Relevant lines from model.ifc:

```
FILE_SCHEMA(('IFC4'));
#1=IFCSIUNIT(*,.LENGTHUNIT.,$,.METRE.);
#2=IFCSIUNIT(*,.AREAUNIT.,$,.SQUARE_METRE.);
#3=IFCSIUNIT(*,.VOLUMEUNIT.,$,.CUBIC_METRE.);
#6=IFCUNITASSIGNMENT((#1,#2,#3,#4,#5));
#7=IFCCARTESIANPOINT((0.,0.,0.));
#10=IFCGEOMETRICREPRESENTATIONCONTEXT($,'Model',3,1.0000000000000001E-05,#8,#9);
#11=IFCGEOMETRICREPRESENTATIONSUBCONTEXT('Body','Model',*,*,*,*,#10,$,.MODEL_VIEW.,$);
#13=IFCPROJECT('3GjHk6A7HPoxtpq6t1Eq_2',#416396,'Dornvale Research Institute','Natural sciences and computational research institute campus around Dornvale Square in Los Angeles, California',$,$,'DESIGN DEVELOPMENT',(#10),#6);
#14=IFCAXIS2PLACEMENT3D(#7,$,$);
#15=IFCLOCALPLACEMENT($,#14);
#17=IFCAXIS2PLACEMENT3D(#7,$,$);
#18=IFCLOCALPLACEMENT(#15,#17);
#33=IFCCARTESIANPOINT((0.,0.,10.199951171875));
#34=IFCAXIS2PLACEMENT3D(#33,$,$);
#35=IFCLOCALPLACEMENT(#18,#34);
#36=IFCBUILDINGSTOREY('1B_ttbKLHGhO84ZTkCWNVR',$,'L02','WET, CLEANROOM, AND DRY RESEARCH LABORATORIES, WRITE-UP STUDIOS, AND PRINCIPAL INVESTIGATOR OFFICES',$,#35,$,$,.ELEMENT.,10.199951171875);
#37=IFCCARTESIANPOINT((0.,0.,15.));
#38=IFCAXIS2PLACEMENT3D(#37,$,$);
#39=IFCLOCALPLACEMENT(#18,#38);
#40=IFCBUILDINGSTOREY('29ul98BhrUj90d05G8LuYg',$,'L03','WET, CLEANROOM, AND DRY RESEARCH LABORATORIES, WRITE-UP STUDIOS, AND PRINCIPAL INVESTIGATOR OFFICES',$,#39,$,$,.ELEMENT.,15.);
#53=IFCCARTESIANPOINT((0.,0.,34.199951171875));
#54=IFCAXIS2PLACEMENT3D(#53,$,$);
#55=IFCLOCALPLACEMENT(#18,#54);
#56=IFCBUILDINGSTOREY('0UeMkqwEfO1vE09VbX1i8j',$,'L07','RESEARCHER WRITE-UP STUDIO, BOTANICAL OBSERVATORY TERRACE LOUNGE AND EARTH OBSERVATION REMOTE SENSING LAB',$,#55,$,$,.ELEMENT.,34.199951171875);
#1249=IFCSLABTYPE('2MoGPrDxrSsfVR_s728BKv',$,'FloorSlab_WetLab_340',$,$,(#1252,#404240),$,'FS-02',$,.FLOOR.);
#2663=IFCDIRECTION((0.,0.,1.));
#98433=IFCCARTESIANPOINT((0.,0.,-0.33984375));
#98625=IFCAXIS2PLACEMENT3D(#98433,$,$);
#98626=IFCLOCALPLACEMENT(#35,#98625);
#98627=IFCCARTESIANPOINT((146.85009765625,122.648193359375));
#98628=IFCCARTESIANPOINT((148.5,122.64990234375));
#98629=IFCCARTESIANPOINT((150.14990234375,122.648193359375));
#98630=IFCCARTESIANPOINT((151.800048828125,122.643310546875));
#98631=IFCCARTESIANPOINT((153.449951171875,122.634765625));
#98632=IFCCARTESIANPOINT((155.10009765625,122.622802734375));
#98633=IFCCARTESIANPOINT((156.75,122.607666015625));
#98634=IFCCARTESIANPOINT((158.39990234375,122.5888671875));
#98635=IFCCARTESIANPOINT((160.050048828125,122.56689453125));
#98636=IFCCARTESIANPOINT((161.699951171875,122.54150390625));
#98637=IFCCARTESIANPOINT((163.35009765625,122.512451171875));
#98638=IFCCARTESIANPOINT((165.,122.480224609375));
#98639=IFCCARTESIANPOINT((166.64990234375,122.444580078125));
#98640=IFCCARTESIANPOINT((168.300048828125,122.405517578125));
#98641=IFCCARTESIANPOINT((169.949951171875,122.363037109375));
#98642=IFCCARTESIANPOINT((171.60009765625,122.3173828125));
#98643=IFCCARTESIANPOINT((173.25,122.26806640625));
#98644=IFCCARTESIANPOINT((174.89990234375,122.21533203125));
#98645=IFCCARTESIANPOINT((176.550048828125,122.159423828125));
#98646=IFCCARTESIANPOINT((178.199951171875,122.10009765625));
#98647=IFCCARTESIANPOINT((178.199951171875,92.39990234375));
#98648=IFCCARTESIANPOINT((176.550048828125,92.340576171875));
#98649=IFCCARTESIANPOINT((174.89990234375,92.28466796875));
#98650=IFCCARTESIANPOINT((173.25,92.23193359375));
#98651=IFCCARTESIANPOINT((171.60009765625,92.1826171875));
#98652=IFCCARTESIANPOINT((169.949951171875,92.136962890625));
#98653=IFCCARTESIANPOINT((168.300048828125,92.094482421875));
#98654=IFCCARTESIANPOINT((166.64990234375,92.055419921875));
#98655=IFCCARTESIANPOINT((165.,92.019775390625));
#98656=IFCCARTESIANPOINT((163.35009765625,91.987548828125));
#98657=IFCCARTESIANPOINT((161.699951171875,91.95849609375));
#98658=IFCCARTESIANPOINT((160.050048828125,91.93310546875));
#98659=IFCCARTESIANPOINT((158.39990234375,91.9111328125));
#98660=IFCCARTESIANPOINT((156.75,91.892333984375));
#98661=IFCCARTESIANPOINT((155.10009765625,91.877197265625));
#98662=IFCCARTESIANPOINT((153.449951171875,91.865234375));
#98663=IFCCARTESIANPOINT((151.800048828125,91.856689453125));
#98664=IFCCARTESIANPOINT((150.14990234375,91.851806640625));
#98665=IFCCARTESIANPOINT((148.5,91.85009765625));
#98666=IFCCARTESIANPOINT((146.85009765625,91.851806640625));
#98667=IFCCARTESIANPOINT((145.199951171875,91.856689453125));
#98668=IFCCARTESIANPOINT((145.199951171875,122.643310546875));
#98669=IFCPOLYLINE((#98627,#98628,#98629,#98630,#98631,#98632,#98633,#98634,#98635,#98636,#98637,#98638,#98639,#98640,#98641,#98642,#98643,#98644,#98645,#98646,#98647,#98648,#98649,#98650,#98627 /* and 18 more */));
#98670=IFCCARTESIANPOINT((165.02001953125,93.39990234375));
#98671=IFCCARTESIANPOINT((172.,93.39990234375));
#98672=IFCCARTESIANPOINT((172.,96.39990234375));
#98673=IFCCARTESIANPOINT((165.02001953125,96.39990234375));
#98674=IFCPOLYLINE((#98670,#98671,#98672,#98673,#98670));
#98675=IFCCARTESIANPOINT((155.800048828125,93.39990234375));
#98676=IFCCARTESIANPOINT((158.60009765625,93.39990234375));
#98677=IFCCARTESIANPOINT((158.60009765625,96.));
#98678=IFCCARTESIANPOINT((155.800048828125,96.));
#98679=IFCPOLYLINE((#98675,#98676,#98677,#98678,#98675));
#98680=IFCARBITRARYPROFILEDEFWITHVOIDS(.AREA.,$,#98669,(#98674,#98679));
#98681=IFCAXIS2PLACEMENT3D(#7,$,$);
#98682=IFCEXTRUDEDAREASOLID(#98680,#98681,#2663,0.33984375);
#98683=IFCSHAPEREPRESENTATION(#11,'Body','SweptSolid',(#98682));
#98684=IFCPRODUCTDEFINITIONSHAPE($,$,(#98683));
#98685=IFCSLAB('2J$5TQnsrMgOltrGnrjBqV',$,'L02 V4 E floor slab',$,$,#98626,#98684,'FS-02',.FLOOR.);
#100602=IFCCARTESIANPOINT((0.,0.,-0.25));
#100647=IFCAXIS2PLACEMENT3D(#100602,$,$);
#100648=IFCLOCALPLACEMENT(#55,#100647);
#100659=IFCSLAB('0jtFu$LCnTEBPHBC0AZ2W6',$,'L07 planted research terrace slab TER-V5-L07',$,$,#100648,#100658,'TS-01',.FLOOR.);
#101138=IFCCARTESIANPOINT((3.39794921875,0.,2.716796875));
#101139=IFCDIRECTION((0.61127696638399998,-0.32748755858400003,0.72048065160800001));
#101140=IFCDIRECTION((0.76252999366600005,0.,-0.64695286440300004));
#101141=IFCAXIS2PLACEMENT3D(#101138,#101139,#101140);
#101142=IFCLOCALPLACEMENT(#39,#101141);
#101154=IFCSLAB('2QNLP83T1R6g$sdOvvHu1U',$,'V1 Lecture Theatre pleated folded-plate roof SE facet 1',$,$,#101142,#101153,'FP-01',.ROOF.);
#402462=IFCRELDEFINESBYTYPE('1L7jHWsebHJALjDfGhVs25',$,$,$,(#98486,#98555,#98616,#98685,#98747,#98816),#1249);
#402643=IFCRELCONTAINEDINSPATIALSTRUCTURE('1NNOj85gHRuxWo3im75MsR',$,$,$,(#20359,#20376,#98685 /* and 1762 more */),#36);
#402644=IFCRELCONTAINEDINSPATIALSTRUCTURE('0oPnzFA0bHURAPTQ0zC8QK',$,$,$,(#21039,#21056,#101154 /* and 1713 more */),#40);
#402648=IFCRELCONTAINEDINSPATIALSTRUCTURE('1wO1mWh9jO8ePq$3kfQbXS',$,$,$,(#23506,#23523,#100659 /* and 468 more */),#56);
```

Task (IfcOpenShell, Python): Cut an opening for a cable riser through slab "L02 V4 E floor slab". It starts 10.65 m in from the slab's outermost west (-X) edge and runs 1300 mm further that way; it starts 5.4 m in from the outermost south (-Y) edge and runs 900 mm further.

```python
import numpy as np
import ifcopenshell
import ifcopenshell.api.feature
import ifcopenshell.api.geometry
import ifcopenshell.api.root
import ifcopenshell.geom
import ifcopenshell.util.placement
import ifcopenshell.util.representation
import ifcopenshell.util.shape
import ifcopenshell.util.unit

model = ifcopenshell.open("model.ifc")
unit_scale = ifcopenshell.util.unit.calculate_unit_scale(model)
settings = ifcopenshell.geom.settings()


def volume(element):
    """Net volume in cubic metres, openings subtracted."""
    shape = ifcopenshell.geom.create_shape(settings, element)
    return ifcopenshell.util.shape.get_volume(shape.geometry)


slab = model.by_id(98685)
before = volume(slab)

# Extent in the slab's own axes, in metres. The edges named are its -X and -Y sides.
slab_shape = ifcopenshell.geom.create_shape(settings, slab)
vertices = ifcopenshell.util.shape.get_vertices(slab_shape.geometry)
x_min, y_min, bottom = vertices.min(axis=0)
top = vertices[:, 2].max()

opening = ifcopenshell.api.root.create_entity(model, ifc_class="IfcOpeningElement", name="Cable riser opening", predefined_type="OPENING")
context = ifcopenshell.util.representation.get_context(model, "Model", "Body", "MODEL_VIEW")
width, depth = 1.3, 0.9
outline = [(0.0, 0.0), (width, 0.0), (width, depth), (0.0, depth), (0.0, 0.0)]
# Overshoot both faces by 50 mm so the cut is clean.
shape = ifcopenshell.api.geometry.add_slab_representation(
    model, context=context, depth=top - bottom + 0.1, polyline=outline
)
ifcopenshell.api.geometry.assign_representation(model, product=opening, representation=shape)

matrix = ifcopenshell.util.placement.get_local_placement(slab.ObjectPlacement)
matrix[:, 3] = matrix @ np.append(np.array([x_min + 10.65, y_min + 5.4, bottom - 0.05]) / unit_scale, 1.0)
ifcopenshell.api.geometry.edit_object_placement(model, product=opening, matrix=matrix, is_si=False)
ifcopenshell.api.feature.add_feature(model, feature=opening, element=slab)

after = volume(slab)

print(f"slab volume {before:.3f} -> {after:.3f} m3")

model.write("model_v2.ifc")
```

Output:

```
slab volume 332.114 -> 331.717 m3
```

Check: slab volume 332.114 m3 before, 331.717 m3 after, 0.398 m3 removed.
